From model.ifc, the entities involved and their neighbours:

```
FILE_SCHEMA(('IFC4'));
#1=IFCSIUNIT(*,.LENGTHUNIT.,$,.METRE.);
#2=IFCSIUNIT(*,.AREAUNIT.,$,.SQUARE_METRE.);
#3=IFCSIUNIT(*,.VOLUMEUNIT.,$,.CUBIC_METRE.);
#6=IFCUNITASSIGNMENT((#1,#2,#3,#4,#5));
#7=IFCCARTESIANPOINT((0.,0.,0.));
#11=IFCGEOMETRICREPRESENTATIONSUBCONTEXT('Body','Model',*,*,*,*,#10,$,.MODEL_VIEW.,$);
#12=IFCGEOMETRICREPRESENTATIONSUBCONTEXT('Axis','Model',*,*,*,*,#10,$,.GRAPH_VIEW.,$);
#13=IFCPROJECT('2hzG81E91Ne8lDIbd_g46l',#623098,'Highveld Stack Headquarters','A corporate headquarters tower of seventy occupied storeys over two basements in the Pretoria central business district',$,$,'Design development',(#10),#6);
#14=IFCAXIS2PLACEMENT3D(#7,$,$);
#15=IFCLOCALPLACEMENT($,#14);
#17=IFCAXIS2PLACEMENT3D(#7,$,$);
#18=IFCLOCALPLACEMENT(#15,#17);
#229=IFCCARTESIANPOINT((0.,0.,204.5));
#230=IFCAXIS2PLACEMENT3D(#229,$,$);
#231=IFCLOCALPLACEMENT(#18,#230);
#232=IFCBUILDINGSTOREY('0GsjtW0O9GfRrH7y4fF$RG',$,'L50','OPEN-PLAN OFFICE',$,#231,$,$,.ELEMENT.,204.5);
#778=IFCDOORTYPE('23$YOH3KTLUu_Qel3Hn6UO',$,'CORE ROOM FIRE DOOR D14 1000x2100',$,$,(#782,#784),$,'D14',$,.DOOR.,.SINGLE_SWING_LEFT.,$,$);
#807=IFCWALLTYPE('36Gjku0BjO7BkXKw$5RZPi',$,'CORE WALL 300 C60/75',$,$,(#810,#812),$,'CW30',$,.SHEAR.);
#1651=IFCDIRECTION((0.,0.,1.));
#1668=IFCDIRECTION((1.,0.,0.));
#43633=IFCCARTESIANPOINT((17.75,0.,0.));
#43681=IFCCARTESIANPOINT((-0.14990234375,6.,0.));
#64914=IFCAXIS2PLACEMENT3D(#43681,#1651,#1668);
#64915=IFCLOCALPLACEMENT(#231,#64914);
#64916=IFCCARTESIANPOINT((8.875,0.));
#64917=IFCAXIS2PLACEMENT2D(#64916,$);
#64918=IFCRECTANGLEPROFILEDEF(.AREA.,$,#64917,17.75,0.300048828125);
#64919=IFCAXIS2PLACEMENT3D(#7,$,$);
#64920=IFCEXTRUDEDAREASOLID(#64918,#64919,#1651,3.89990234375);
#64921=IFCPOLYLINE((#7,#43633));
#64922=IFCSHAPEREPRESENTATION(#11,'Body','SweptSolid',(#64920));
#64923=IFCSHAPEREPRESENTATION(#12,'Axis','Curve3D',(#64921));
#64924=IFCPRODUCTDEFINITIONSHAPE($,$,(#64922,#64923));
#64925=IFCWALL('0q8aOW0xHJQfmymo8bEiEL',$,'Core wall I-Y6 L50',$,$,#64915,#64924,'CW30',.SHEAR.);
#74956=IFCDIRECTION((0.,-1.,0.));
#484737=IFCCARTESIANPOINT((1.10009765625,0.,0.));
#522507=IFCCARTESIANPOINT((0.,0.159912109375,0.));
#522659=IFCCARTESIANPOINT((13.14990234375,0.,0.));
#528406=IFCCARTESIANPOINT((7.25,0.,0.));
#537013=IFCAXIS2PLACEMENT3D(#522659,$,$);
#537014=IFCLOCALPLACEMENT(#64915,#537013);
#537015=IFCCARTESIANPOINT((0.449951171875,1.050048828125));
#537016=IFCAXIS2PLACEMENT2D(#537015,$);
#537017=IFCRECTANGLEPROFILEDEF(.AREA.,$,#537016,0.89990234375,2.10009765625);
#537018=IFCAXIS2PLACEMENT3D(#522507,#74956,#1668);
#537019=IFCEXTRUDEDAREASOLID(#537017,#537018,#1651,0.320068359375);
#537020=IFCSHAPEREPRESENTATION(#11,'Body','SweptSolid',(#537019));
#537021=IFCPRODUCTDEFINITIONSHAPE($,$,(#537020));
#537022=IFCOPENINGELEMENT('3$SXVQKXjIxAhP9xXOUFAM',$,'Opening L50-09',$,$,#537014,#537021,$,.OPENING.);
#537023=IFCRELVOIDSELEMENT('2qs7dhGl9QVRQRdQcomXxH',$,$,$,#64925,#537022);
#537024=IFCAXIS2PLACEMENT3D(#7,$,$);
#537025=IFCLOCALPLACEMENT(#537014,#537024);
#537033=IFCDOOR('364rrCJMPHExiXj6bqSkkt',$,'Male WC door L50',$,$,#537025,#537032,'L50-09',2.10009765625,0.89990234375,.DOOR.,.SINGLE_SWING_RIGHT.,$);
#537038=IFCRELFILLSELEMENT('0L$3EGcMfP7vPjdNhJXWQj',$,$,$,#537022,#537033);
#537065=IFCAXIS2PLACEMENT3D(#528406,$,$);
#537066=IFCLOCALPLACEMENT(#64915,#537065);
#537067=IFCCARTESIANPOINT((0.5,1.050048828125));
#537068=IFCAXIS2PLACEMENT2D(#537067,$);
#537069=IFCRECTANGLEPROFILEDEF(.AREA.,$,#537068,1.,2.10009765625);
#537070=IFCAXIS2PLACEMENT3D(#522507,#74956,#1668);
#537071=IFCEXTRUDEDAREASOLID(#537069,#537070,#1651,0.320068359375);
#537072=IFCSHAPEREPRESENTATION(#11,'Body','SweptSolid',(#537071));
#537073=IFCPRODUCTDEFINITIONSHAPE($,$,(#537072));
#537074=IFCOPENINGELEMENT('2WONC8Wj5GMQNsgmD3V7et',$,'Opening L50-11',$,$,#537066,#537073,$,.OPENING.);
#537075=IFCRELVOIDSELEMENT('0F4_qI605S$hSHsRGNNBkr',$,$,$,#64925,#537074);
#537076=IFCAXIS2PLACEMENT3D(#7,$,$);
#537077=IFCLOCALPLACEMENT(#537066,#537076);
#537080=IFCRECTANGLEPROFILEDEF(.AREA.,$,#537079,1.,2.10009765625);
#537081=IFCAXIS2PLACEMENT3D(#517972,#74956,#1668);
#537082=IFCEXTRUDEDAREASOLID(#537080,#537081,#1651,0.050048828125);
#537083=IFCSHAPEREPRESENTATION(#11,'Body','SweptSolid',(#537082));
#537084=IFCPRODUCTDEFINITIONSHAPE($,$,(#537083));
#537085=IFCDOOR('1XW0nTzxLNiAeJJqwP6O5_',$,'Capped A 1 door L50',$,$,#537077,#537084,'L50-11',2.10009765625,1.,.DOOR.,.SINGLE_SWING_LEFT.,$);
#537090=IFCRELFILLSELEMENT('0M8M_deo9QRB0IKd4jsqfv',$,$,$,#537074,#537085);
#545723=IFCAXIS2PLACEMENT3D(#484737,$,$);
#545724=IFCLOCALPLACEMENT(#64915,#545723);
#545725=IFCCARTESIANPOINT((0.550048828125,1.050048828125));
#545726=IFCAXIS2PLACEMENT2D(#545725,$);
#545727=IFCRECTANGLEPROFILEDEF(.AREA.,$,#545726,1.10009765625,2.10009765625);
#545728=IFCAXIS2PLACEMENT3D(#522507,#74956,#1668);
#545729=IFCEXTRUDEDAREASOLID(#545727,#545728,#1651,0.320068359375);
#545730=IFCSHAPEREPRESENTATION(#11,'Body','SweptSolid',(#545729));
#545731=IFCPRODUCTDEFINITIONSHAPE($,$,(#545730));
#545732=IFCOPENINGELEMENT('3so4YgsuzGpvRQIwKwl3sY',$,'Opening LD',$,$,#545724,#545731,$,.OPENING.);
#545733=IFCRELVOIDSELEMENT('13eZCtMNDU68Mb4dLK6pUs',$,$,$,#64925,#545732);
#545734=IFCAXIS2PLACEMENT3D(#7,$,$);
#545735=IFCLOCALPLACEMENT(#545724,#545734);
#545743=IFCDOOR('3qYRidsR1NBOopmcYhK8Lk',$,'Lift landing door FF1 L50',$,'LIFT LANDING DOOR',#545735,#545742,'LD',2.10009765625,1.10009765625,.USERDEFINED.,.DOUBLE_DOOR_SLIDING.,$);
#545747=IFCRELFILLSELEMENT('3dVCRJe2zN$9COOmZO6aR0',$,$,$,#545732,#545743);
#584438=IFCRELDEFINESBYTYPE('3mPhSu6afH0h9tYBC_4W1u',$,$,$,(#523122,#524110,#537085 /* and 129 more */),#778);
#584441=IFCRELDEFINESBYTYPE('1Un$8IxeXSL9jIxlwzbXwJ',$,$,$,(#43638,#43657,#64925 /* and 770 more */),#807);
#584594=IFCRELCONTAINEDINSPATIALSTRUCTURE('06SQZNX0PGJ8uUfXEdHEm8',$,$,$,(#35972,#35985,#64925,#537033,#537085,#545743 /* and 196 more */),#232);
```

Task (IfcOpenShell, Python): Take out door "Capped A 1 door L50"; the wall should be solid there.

```python
import ifcopenshell
import ifcopenshell.api.feature
import ifcopenshell.api.root
import ifcopenshell.geom
import ifcopenshell.util.shape

model = ifcopenshell.open("model.ifc")
settings = ifcopenshell.geom.settings()


def volume(element):
    """Net volume in cubic metres, openings subtracted."""
    shape = ifcopenshell.geom.create_shape(settings, element)
    return ifcopenshell.util.shape.get_volume(shape.geometry)


door = model.by_guid("1XW0nTzxLNiAeJJqwP6O5_")
opening = door.FillsVoids[0].RelatingOpeningElement
wall = opening.VoidsElements[0].RelatingBuildingElement
before = volume(wall)

ifcopenshell.api.root.remove_product(model, product=door)
ifcopenshell.api.feature.remove_feature(model, feature=opening)

after = volume(wall)

print(f"wall volume {before:.3f} -> {after:.3f} m3")

model.write("model_v2.ifc")
```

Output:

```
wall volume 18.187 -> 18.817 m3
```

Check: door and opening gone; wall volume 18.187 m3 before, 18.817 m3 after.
